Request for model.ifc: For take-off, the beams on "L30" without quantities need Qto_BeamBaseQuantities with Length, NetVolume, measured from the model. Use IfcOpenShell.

First a look at what the model holds.

```python
import ifcopenshell
import ifcopenshell.util.element
import ifcopenshell.util.unit

model = ifcopenshell.open("model.ifc")
print(model.schema)
for unit_type in ("LENGTHUNIT", "AREAUNIT", "VOLUMEUNIT"):
    print(unit_type, ifcopenshell.util.unit.calculate_unit_scale(model, unit_type))
storey = next(s for s in model.by_type("IfcBuildingStorey") if s.Name == "L30")
beams = [e for e in ifcopenshell.util.element.get_decomposition(storey) if e.is_a("IfcBeam")]
for e in sorted(beams, key=lambda e: e.id()):
    print(e.id(), e.is_a(), e.Name, list(ifcopenshell.util.element.get_psets(e, qtos_only=True)), sep=" | ")
```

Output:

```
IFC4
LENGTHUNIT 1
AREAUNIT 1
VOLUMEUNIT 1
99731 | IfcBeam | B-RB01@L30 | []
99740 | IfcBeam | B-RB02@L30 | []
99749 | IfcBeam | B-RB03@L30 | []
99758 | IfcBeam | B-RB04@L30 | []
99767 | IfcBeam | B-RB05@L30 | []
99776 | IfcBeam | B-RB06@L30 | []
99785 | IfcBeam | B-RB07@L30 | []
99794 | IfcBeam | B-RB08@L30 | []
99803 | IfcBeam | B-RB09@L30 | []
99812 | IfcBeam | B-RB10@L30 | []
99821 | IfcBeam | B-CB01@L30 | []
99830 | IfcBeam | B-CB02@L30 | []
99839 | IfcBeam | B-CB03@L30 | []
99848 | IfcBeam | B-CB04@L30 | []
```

```python
import ifcopenshell
import ifcopenshell.api.pset
import ifcopenshell.geom
import ifcopenshell.util.element
import ifcopenshell.util.shape
import ifcopenshell.util.unit

model = ifcopenshell.open("model.ifc")
unit_scale = ifcopenshell.util.unit.calculate_unit_scale(model)
volume_scale = ifcopenshell.util.unit.calculate_unit_scale(model, "VOLUMEUNIT")
settings = ifcopenshell.geom.settings()

storey = next(s for s in model.by_type("IfcBuildingStorey") if s.Name == "L30")
beams = [e for e in ifcopenshell.util.element.get_decomposition(storey) if e.is_a("IfcBeam")]

for e in sorted(beams, key=lambda e: e.id()):
    if ifcopenshell.util.element.get_psets(e, qtos_only=True, should_inherit=False):
        continue
    # Geometry comes back in metres, in the element's own axes.
    shape = ifcopenshell.geom.create_shape(settings, e)
    values = {
        "Length": ifcopenshell.util.shape.get_max_xyz(shape.geometry) / unit_scale,
        "NetVolume": ifcopenshell.util.shape.get_volume(shape.geometry) / volume_scale,
    }
    qto = ifcopenshell.api.pset.add_qto(model, product=e, name="Qto_BeamBaseQuantities")
    ifcopenshell.api.pset.edit_qto(model, qto=qto, properties=values)
    print(e.id(), {k: round(v, 3) for k, v in values.items()})

model.write("model_v2.ifc")
```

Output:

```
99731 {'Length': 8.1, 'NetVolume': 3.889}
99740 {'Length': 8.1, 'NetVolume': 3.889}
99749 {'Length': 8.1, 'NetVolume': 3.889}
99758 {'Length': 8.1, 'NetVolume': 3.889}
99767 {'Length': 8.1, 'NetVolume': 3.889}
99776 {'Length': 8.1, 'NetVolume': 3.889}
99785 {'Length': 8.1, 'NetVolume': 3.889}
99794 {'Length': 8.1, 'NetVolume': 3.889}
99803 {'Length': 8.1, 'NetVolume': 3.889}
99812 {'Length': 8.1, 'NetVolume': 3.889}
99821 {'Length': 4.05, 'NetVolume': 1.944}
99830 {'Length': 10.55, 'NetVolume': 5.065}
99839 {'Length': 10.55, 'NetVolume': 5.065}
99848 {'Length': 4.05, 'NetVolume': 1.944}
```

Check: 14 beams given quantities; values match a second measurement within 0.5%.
